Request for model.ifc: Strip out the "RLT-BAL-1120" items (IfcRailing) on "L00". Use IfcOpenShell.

First a look at what the model holds.

```python
import ifcopenshell
import ifcopenshell.util.element

model = ifcopenshell.open("model.ifc")
print(model.schema)
storey = next(s for s in model.by_type("IfcBuildingStorey") if s.Name == "L00")
railings = [e for e in ifcopenshell.util.element.get_decomposition(storey) if e.is_a("IfcRailing")]
seen = {}
for e in railings:
    element_type = ifcopenshell.util.element.get_type(e)
    name = element_type.Name if element_type not in (None, e) else None
    seen[name] = seen.get(name, 0) + 1
for name, count in sorted(seen.items(), key=str):
    print(count, "x", name)
```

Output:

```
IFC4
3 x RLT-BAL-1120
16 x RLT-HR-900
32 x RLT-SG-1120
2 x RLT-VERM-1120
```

```python
import ifcopenshell
import ifcopenshell.api.root
import ifcopenshell.util.element

model = ifcopenshell.open("model.ifc")

storey = next(s for s in model.by_type("IfcBuildingStorey") if s.Name == "L00")
railings = [e for e in ifcopenshell.util.element.get_decomposition(storey) if e.is_a("IfcRailing")]
targets = [e for e in railings if (t := ifcopenshell.util.element.get_type(e)) not in (None, e) and t.Name == "RLT-BAL-1120"]

for e in targets:
    ifcopenshell.api.root.remove_product(model, product=e)
print(len(targets), "removed")

model.write("model-out.ifc")
```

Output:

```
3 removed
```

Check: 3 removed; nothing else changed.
